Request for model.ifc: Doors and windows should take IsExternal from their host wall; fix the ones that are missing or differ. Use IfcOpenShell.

First a look at what the model holds.

```python
import ifcopenshell
import ifcopenshell.util.element

model = ifcopenshell.open("model.ifc")
print(model.schema)
seen = {}
for e in model.by_type("IfcDoor") + model.by_type("IfcWindow"):
    if not e.FillsVoids:
        continue
    host = e.FillsVoids[0].RelatingOpeningElement.VoidsElements[0].RelatingBuildingElement
    own = ifcopenshell.util.element.get_pset(e, f"Pset_{e.is_a()[3:].removesuffix('StandardCase')}Common", "IsExternal")
    wall = ifcopenshell.util.element.get_pset(host, "Pset_WallCommon", "IsExternal")
    seen[e.is_a(), own, wall] = seen.get((e.is_a(), own, wall), 0) + 1
for (cls, own, wall), count in sorted(seen.items(), key=str):
    print(count, cls, "IsExternal:", own, "| host wall:", wall)
```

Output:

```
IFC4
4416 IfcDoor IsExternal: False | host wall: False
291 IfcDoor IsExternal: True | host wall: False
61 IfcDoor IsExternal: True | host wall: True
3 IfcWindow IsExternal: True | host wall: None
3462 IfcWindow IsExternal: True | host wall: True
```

```python
import ifcopenshell
import ifcopenshell.api.pset
import ifcopenshell.util.element

model = ifcopenshell.open("model.ifc")

count = 0
for ifc_class, pset_name in (("IfcDoor", "Pset_DoorCommon"), ("IfcWindow", "Pset_WindowCommon")):
    for e in model.by_type(ifc_class):
        if not e.FillsVoids:
            continue
        host = e.FillsVoids[0].RelatingOpeningElement.VoidsElements[0].RelatingBuildingElement
        external = ifcopenshell.util.element.get_pset(host, "Pset_WallCommon", "IsExternal")
        if external is None or ifcopenshell.util.element.get_pset(e, pset_name, "IsExternal") == external:
            continue
        found = ifcopenshell.util.element.get_pset(e, pset_name, should_inherit=False)
        if found:
            pset = model.by_id(found["id"])
            if len(ifcopenshell.util.element.get_elements_by_pset(pset)) > 1:
                pset = ifcopenshell.api.pset.unshare_pset(model, products=[e], pset=pset)[0]
        else:
            pset = ifcopenshell.api.pset.add_pset(model, product=e, name=pset_name)
        ifcopenshell.api.pset.edit_pset(model, pset=pset, properties={"IsExternal": external})
        count += 1

print(count, "updated")

model.write("model-out.ifc")
```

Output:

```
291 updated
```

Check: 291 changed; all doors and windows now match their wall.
